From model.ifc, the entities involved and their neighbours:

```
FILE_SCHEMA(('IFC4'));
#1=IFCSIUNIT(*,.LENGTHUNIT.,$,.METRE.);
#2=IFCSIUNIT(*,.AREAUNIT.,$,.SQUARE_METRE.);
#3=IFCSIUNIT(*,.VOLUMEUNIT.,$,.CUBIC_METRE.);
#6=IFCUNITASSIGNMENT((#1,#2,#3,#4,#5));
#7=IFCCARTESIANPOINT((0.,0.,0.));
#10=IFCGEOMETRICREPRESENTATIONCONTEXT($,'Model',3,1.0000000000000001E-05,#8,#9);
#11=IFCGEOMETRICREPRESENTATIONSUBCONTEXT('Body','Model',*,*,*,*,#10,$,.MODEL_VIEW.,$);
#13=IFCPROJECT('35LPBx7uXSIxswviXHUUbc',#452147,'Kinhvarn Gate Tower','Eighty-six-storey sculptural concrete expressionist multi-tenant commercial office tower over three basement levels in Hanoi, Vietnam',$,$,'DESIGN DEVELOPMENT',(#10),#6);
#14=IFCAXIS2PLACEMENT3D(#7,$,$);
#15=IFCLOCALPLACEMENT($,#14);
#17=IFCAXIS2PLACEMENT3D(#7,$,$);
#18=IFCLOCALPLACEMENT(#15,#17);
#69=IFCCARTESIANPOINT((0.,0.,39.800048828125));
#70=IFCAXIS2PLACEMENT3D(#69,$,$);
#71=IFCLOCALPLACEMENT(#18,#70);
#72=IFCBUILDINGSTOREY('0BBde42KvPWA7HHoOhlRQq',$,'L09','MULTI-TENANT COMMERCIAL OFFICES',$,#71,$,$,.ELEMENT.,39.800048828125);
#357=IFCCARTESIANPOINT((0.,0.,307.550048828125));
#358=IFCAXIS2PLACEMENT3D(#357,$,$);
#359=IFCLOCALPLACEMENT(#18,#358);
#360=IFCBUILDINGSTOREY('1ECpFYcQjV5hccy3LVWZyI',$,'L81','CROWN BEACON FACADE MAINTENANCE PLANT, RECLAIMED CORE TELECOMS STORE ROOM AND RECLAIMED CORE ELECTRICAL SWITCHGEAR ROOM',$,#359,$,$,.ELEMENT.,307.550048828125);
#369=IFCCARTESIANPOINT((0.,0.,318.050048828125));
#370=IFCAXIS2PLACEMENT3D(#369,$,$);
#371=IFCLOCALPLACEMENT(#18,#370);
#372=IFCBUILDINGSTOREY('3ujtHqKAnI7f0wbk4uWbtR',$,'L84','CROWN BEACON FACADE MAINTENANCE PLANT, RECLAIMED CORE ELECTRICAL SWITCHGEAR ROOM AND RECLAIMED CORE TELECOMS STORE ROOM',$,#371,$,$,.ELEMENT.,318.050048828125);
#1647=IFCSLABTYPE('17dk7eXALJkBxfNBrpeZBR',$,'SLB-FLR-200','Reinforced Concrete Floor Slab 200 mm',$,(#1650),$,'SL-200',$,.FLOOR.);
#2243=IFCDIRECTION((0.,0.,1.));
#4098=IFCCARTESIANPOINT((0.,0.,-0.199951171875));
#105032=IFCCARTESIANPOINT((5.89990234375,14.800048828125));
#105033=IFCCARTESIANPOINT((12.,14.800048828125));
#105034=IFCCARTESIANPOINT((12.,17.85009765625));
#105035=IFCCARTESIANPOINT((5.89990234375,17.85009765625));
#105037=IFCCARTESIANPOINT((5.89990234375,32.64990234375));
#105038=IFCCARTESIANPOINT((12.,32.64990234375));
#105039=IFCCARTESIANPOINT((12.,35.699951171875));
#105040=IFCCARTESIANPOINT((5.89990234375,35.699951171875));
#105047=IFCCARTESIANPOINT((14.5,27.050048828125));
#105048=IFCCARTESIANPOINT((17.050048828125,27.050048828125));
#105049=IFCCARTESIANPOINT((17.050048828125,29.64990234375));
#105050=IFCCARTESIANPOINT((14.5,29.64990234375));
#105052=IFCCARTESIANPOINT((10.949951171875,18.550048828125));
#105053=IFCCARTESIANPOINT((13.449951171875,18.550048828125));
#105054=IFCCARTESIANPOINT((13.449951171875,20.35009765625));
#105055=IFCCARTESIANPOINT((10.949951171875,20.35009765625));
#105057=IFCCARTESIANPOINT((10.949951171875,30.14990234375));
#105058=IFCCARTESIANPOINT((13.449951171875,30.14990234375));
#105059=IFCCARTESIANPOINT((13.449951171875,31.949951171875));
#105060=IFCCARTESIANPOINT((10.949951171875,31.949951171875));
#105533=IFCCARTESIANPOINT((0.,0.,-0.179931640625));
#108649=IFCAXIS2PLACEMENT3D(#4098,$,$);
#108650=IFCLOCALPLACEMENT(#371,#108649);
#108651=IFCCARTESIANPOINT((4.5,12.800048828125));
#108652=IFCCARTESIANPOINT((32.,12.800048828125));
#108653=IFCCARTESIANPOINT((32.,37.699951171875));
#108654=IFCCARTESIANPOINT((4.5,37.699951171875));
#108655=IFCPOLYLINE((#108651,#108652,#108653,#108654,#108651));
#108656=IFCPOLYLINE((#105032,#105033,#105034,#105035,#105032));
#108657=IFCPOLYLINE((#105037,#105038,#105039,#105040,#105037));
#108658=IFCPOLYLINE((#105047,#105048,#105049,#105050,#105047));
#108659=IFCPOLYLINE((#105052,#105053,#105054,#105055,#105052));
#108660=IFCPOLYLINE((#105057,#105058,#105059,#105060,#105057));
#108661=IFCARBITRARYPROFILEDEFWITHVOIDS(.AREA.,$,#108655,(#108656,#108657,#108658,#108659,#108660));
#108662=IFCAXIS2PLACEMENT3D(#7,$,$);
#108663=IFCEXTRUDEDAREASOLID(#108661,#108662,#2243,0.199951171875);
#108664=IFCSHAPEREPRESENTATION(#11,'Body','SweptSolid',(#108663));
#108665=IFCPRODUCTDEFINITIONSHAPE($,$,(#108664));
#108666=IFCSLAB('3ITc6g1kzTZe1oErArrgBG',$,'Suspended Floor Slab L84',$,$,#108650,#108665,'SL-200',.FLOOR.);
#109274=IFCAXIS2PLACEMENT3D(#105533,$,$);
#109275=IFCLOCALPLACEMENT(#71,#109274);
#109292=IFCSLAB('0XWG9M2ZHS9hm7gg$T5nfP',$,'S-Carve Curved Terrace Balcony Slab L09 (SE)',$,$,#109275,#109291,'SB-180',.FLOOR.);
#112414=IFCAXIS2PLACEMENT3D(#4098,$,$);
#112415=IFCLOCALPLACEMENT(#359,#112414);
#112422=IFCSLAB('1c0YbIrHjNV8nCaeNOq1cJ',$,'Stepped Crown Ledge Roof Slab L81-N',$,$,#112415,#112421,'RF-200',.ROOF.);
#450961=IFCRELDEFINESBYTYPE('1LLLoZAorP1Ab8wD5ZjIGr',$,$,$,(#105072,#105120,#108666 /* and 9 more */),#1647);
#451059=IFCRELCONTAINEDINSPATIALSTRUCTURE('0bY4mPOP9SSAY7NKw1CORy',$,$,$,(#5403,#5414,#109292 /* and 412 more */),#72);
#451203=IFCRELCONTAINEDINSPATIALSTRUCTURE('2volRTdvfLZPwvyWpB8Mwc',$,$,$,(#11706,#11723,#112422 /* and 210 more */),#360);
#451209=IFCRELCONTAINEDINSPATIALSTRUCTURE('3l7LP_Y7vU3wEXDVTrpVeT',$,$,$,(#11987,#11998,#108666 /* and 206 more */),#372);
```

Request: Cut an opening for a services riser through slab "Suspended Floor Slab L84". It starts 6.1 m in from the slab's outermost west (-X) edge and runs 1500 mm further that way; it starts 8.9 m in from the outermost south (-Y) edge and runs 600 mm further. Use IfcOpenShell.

```python
import numpy as np
import ifcopenshell
import ifcopenshell.api.feature
import ifcopenshell.api.geometry
import ifcopenshell.api.root
import ifcopenshell.geom
import ifcopenshell.util.placement
import ifcopenshell.util.representation
import ifcopenshell.util.shape
import ifcopenshell.util.unit

model = ifcopenshell.open("model.ifc")
unit_scale = ifcopenshell.util.unit.calculate_unit_scale(model)
settings = ifcopenshell.geom.settings()


def volume(element):
    """Net volume in cubic metres, openings subtracted."""
    shape = ifcopenshell.geom.create_shape(settings, element)
    return ifcopenshell.util.shape.get_volume(shape.geometry)


slab = model.by_guid("3ITc6g1kzTZe1oErArrgBG")
before = volume(slab)

# Extent in the slab's own axes, in metres. The edges named are its -X and -Y sides.
slab_shape = ifcopenshell.geom.create_shape(settings, slab)
vertices = ifcopenshell.util.shape.get_vertices(slab_shape.geometry)
x_min, y_min, bottom = vertices.min(axis=0)
top = vertices[:, 2].max()

opening = ifcopenshell.api.root.create_entity(model, ifc_class="IfcOpeningElement", name="Services riser opening", predefined_type="OPENING")
context = ifcopenshell.util.representation.get_context(model, "Model", "Body", "MODEL_VIEW")
width, depth = 1.5, 0.6
outline = [(0.0, 0.0), (width, 0.0), (width, depth), (0.0, depth), (0.0, 0.0)]
# Overshoot both faces by 50 mm so the cut is clean.
shape = ifcopenshell.api.geometry.add_slab_representation(
    model, context=context, depth=top - bottom + 0.1, polyline=outline
)
ifcopenshell.api.geometry.assign_representation(model, product=opening, representation=shape)

matrix = ifcopenshell.util.placement.get_local_placement(slab.ObjectPlacement)
matrix[:, 3] = matrix @ np.append(np.array([x_min + 6.1, y_min + 8.9, bottom - 0.05]) / unit_scale, 1.0)
ifcopenshell.api.geometry.edit_object_placement(model, product=opening, matrix=matrix, is_si=False)
ifcopenshell.api.feature.add_feature(model, feature=opening, element=slab)

after = volume(slab)

print(f"slab volume {before:.3f} -> {after:.3f} m3")

model.write("model_edited.ifc")
```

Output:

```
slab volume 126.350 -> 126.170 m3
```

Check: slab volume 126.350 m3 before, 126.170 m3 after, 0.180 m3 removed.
